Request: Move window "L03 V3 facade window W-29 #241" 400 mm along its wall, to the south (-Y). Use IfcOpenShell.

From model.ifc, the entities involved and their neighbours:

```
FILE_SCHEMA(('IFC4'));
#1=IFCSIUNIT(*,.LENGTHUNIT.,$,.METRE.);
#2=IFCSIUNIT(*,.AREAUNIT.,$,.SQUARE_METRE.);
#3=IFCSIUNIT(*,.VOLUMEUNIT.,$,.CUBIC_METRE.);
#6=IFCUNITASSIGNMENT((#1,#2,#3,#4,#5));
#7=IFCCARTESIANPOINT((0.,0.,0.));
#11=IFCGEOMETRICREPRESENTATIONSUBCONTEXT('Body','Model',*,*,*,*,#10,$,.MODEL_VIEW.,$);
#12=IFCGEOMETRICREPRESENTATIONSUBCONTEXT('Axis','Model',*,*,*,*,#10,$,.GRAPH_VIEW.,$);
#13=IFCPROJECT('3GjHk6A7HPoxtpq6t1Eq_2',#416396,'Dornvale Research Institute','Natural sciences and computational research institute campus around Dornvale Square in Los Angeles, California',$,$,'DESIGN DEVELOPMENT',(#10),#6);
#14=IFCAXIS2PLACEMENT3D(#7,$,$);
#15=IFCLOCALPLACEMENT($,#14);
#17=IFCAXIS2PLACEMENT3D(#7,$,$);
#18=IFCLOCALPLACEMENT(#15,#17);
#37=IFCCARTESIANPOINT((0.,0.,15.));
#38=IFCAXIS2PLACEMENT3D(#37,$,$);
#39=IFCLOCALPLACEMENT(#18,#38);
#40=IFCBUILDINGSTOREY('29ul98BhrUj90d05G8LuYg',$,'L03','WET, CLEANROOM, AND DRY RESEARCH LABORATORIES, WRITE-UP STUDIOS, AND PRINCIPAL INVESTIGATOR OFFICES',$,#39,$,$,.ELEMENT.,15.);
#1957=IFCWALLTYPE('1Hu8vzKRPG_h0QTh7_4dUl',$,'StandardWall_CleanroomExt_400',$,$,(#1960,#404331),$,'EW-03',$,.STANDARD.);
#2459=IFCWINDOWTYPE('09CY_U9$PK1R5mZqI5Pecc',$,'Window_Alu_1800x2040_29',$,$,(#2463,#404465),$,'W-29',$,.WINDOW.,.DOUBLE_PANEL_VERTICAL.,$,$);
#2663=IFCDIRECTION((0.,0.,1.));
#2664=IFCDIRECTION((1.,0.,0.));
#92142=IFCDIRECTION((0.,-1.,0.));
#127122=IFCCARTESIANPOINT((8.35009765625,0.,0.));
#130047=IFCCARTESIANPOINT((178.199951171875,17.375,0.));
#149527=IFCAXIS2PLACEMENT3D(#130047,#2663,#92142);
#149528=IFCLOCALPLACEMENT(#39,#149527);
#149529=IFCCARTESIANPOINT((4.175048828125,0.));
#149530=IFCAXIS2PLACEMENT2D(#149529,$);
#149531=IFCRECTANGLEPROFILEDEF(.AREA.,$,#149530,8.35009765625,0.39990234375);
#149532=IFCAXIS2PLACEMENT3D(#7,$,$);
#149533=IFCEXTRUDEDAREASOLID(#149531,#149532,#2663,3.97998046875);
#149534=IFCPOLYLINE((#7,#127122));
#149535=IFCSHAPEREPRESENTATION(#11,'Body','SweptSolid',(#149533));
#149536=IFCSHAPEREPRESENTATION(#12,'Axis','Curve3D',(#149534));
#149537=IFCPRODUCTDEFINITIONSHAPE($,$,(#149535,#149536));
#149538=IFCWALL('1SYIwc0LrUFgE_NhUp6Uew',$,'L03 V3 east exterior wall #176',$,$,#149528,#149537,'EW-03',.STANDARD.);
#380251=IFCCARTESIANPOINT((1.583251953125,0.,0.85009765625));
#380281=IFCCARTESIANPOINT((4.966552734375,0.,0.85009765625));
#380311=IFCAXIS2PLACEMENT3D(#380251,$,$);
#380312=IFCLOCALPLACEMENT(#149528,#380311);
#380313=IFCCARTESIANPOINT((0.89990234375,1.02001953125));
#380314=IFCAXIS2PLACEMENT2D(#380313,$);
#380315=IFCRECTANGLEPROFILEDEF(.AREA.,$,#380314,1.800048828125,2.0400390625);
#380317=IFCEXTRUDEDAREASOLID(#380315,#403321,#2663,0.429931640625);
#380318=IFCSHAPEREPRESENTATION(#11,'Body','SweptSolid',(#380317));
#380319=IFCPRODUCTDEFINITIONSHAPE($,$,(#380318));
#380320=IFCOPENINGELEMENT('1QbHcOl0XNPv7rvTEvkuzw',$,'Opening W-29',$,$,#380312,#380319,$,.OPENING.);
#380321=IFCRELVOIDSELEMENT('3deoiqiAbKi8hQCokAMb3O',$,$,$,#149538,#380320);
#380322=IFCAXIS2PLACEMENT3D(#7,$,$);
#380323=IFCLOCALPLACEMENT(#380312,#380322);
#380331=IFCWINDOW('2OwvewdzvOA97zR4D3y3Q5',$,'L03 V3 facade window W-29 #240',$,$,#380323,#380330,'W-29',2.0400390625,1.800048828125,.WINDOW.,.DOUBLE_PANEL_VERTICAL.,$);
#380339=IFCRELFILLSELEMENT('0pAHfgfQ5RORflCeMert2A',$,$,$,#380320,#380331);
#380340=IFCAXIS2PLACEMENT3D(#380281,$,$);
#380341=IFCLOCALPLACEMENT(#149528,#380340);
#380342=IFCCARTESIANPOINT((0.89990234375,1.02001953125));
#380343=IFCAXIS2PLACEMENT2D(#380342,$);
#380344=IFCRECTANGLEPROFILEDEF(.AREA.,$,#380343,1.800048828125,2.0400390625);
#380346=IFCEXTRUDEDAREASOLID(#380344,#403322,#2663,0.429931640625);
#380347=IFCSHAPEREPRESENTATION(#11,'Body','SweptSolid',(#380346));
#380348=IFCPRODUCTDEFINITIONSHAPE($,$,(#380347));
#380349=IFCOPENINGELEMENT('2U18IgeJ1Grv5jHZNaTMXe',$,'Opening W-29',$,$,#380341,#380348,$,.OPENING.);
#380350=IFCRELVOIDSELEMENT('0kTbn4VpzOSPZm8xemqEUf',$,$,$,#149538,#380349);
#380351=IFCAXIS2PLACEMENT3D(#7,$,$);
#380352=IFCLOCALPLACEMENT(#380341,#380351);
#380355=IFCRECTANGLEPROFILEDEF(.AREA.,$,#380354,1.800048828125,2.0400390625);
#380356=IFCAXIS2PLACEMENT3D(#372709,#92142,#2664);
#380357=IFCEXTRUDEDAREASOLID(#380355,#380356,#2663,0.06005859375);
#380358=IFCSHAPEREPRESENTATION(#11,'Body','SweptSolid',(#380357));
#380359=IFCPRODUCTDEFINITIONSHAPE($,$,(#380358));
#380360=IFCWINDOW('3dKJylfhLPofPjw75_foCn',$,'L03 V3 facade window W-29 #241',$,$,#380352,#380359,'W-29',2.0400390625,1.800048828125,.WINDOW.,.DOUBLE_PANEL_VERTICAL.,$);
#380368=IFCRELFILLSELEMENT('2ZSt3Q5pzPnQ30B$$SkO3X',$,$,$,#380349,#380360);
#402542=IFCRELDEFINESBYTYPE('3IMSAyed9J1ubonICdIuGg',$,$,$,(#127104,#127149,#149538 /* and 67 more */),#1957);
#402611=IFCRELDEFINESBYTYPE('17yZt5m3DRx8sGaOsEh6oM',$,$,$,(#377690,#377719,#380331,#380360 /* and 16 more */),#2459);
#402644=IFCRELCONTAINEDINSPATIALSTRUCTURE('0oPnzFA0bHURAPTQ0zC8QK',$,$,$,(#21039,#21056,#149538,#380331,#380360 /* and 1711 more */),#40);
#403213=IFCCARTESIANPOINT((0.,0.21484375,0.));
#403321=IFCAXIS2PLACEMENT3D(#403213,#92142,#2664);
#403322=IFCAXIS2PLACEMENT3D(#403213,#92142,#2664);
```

```python
import ifcopenshell
import ifcopenshell.api.geometry
import ifcopenshell.util.placement

model = ifcopenshell.open("model.ifc")

window = model.by_guid("3dKJylfhLPofPjw75_foCn")
opening = window.FillsVoids[0].RelatingOpeningElement
wall = opening.VoidsElements[0].RelatingBuildingElement

wall_matrix = ifcopenshell.util.placement.get_local_placement(wall.ObjectPlacement)
shift = wall_matrix[:3, 0] * 0.4
before = ifcopenshell.util.placement.get_local_placement(window.ObjectPlacement)[:3, 3].copy()

# The window is placed relative to its opening, so it follows when the opening moves.
matrix = ifcopenshell.util.placement.get_local_placement(opening.ObjectPlacement)
matrix[:3, 3] += shift
ifcopenshell.api.geometry.edit_object_placement(
    model, product=opening, matrix=matrix, is_si=False, should_transform_children=True
)

after = ifcopenshell.util.placement.get_local_placement(window.ObjectPlacement)[:3, 3]
print("window moved by", (after - before).round(3) + 0.0)

model.write("model-out.ifc")
```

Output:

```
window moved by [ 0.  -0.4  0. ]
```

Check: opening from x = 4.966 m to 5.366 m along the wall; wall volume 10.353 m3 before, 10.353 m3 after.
